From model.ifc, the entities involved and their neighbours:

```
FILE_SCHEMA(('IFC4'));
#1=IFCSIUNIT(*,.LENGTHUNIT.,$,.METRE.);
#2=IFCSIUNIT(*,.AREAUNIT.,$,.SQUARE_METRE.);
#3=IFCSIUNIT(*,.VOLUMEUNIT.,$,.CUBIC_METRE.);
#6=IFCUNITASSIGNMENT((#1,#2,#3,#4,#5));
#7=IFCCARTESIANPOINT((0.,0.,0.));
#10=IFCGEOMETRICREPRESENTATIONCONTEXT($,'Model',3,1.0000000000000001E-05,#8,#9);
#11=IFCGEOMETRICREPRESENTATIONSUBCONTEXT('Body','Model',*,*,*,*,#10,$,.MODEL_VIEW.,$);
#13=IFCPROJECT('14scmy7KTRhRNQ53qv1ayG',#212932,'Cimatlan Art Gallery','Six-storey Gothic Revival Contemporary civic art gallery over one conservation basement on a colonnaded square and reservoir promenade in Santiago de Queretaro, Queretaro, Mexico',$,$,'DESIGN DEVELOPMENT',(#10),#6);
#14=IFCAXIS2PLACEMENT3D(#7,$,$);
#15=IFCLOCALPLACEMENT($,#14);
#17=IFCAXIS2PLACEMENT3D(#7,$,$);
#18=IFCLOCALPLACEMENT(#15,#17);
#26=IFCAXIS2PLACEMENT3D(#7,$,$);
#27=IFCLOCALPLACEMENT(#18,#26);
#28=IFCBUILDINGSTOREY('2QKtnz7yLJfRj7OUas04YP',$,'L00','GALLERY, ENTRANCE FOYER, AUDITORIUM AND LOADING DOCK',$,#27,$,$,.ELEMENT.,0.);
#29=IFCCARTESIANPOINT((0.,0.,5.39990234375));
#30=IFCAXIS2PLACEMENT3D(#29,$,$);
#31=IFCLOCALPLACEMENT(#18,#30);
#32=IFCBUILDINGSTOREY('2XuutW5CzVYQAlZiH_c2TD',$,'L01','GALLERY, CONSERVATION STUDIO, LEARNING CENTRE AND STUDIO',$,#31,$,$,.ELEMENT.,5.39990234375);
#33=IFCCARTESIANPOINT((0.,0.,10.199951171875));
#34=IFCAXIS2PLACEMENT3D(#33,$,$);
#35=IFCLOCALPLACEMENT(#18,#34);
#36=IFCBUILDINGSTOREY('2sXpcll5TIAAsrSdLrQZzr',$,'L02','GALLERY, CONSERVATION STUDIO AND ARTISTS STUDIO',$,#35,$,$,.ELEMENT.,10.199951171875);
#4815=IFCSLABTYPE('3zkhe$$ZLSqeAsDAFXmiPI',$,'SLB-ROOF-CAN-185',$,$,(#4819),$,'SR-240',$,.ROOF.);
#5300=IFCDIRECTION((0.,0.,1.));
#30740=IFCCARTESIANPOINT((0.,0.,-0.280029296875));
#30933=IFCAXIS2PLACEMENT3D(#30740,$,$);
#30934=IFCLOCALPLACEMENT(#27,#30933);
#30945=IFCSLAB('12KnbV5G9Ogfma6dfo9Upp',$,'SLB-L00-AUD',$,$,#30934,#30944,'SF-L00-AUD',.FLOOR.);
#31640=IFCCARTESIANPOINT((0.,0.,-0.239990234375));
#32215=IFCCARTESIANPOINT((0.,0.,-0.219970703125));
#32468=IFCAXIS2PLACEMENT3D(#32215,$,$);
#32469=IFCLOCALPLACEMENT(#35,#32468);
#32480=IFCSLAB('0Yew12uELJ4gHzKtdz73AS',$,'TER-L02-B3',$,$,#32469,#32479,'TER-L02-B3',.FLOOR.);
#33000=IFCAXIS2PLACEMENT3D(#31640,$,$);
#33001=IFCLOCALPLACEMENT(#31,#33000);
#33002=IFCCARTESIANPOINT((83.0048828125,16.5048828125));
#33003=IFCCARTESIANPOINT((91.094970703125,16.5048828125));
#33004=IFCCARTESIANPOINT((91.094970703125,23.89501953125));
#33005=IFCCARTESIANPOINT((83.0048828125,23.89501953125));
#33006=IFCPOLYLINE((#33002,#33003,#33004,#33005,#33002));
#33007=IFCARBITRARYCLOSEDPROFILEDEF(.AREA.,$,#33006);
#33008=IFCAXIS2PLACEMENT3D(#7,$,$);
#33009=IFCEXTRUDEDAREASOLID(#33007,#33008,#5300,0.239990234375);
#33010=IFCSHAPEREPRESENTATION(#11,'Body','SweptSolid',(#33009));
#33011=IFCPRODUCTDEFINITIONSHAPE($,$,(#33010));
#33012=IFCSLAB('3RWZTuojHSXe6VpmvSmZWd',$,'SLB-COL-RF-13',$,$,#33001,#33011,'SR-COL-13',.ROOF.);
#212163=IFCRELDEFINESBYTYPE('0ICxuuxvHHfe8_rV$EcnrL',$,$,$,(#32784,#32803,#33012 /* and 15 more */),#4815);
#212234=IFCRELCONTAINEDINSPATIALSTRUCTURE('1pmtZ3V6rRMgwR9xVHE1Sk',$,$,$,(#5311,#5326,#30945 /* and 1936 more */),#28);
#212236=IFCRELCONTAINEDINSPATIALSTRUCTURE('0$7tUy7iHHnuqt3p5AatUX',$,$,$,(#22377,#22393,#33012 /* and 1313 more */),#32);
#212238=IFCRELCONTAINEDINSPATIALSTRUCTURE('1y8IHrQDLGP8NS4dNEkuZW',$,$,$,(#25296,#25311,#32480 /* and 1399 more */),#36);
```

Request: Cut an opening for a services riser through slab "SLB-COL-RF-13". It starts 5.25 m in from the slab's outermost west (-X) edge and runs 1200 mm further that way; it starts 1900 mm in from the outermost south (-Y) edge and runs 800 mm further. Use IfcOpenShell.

```python
import numpy as np
import ifcopenshell
import ifcopenshell.api.feature
import ifcopenshell.api.geometry
import ifcopenshell.api.root
import ifcopenshell.geom
import ifcopenshell.util.placement
import ifcopenshell.util.representation
import ifcopenshell.util.shape
import ifcopenshell.util.unit

model = ifcopenshell.open("model.ifc")
unit_scale = ifcopenshell.util.unit.calculate_unit_scale(model)
settings = ifcopenshell.geom.settings()


def volume(element):
    """Net volume in cubic metres, openings subtracted."""
    shape = ifcopenshell.geom.create_shape(settings, element)
    return ifcopenshell.util.shape.get_volume(shape.geometry)


slab = model.by_guid("3RWZTuojHSXe6VpmvSmZWd")
before = volume(slab)

# Extent in the slab's own axes, in metres. The edges named are its -X and -Y sides.
slab_shape = ifcopenshell.geom.create_shape(settings, slab)
vertices = ifcopenshell.util.shape.get_vertices(slab_shape.geometry)
x_min, y_min, bottom = vertices.min(axis=0)
top = vertices[:, 2].max()

opening = ifcopenshell.api.root.create_entity(model, ifc_class="IfcOpeningElement", name="Services riser opening", predefined_type="OPENING")
context = ifcopenshell.util.representation.get_context(model, "Model", "Body", "MODEL_VIEW")
width, depth = 1.2, 0.8
outline = [(0.0, 0.0), (width, 0.0), (width, depth), (0.0, depth), (0.0, 0.0)]
# Overshoot both faces by 50 mm so the cut is clean.
shape = ifcopenshell.api.geometry.add_slab_representation(
    model, context=context, depth=top - bottom + 0.1, polyline=outline
)
ifcopenshell.api.geometry.assign_representation(model, product=opening, representation=shape)

matrix = ifcopenshell.util.placement.get_local_placement(slab.ObjectPlacement)
matrix[:, 3] = matrix @ np.append(np.array([x_min + 5.25, y_min + 1.9, bottom - 0.05]) / unit_scale, 1.0)
ifcopenshell.api.geometry.edit_object_placement(model, product=opening, matrix=matrix, is_si=False)
ifcopenshell.api.feature.add_feature(model, feature=opening, element=slab)

after = volume(slab)

print(f"slab volume {before:.3f} -> {after:.3f} m3")

model.write("model-out.ifc")
```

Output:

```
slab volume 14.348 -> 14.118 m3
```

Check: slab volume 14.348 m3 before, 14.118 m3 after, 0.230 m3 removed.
